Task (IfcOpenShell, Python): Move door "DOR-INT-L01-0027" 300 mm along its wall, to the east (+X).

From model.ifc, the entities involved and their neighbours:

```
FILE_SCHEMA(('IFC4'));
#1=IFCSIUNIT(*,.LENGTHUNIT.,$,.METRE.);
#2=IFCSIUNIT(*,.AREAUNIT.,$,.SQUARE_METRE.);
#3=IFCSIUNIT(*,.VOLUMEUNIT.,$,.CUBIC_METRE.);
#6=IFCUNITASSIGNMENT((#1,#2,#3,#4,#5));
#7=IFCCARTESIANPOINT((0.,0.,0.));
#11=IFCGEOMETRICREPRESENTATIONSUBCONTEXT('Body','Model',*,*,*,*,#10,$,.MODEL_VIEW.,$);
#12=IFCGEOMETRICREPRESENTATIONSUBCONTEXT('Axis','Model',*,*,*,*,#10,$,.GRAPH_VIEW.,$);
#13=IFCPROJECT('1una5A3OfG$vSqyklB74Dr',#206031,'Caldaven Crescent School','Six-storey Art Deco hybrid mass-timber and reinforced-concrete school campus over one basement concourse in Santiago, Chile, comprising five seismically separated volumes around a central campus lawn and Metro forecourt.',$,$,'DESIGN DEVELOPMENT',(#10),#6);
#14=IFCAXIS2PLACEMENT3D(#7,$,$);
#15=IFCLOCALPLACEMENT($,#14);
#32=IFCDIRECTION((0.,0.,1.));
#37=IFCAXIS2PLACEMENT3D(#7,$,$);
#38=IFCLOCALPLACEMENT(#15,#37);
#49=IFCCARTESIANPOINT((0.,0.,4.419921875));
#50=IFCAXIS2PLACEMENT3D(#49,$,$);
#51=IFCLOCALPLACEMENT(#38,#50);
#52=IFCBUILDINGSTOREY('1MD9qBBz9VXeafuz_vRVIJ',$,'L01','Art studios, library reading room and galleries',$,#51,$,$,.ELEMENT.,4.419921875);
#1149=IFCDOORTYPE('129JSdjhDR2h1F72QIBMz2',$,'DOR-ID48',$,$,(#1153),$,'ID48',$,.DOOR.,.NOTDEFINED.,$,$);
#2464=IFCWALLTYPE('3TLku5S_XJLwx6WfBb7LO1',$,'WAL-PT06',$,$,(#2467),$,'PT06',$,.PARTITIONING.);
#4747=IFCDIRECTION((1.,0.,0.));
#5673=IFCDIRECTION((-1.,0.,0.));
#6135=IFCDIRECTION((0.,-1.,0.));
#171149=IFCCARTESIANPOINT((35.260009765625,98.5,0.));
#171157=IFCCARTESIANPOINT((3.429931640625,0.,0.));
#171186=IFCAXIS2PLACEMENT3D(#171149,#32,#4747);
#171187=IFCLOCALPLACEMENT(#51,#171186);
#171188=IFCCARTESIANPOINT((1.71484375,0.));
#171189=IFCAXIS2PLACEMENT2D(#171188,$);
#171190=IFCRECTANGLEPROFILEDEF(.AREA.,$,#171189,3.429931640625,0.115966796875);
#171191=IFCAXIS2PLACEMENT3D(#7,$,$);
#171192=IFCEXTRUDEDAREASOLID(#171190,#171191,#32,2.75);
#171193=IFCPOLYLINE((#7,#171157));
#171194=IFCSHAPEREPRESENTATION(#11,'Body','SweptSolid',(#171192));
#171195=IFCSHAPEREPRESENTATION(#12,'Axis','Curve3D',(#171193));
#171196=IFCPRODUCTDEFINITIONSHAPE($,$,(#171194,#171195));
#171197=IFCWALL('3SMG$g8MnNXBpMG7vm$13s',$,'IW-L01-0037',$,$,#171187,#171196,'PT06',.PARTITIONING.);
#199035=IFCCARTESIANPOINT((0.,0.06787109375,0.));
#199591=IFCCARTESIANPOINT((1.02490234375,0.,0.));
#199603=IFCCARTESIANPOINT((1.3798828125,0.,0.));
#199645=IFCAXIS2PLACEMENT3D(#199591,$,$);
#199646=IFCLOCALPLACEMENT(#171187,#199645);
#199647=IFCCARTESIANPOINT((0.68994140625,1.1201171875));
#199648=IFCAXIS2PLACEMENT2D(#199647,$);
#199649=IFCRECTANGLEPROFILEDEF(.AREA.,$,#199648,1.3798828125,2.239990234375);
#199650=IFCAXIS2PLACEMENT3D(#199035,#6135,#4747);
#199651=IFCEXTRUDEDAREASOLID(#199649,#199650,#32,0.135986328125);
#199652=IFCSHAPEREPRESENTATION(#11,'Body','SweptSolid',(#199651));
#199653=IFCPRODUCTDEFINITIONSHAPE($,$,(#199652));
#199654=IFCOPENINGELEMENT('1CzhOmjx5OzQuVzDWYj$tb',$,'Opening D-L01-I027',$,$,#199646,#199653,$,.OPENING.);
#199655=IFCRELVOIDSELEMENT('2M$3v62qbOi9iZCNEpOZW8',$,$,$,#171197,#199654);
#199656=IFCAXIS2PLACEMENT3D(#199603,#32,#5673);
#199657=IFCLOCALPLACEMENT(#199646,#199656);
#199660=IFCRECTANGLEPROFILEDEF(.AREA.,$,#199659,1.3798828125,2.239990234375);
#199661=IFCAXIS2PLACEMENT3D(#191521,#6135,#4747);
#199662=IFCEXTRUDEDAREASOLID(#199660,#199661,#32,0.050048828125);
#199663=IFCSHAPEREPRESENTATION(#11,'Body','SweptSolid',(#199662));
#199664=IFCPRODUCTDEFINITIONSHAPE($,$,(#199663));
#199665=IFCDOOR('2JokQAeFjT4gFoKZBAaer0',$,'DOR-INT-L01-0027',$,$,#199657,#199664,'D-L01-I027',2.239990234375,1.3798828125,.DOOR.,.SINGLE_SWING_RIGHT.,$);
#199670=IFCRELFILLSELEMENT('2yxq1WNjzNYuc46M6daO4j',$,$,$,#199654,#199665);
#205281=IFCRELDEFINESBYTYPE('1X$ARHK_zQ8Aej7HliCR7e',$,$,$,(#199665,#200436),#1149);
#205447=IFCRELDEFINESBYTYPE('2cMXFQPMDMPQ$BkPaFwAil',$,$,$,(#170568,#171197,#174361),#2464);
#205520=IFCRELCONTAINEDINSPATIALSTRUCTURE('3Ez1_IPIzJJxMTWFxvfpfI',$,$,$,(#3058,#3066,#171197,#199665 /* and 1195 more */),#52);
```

```python
import ifcopenshell
import ifcopenshell.api.geometry
import ifcopenshell.util.placement
import ifcopenshell.util.unit

model = ifcopenshell.open("model.ifc")
unit_scale = ifcopenshell.util.unit.calculate_unit_scale(model)

door = model.by_guid("2JokQAeFjT4gFoKZBAaer0")
opening = door.FillsVoids[0].RelatingOpeningElement
wall = opening.VoidsElements[0].RelatingBuildingElement

wall_matrix = ifcopenshell.util.placement.get_local_placement(wall.ObjectPlacement)
shift = wall_matrix[:3, 0] * 0.3 / unit_scale
before = ifcopenshell.util.placement.get_local_placement(door.ObjectPlacement)[:3, 3].copy()

# The door is placed relative to its opening, so it follows when the opening moves.
matrix = ifcopenshell.util.placement.get_local_placement(opening.ObjectPlacement)
matrix[:3, 3] += shift
ifcopenshell.api.geometry.edit_object_placement(
    model, product=opening, matrix=matrix, is_si=False, should_transform_children=True
)

after = ifcopenshell.util.placement.get_local_placement(door.ObjectPlacement)[:3, 3]
print("door moved by", (after - before).round(3) + 0.0)

model.write("model-out.ifc")
```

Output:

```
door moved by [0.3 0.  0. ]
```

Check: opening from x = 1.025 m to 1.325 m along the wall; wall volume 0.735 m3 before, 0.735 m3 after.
